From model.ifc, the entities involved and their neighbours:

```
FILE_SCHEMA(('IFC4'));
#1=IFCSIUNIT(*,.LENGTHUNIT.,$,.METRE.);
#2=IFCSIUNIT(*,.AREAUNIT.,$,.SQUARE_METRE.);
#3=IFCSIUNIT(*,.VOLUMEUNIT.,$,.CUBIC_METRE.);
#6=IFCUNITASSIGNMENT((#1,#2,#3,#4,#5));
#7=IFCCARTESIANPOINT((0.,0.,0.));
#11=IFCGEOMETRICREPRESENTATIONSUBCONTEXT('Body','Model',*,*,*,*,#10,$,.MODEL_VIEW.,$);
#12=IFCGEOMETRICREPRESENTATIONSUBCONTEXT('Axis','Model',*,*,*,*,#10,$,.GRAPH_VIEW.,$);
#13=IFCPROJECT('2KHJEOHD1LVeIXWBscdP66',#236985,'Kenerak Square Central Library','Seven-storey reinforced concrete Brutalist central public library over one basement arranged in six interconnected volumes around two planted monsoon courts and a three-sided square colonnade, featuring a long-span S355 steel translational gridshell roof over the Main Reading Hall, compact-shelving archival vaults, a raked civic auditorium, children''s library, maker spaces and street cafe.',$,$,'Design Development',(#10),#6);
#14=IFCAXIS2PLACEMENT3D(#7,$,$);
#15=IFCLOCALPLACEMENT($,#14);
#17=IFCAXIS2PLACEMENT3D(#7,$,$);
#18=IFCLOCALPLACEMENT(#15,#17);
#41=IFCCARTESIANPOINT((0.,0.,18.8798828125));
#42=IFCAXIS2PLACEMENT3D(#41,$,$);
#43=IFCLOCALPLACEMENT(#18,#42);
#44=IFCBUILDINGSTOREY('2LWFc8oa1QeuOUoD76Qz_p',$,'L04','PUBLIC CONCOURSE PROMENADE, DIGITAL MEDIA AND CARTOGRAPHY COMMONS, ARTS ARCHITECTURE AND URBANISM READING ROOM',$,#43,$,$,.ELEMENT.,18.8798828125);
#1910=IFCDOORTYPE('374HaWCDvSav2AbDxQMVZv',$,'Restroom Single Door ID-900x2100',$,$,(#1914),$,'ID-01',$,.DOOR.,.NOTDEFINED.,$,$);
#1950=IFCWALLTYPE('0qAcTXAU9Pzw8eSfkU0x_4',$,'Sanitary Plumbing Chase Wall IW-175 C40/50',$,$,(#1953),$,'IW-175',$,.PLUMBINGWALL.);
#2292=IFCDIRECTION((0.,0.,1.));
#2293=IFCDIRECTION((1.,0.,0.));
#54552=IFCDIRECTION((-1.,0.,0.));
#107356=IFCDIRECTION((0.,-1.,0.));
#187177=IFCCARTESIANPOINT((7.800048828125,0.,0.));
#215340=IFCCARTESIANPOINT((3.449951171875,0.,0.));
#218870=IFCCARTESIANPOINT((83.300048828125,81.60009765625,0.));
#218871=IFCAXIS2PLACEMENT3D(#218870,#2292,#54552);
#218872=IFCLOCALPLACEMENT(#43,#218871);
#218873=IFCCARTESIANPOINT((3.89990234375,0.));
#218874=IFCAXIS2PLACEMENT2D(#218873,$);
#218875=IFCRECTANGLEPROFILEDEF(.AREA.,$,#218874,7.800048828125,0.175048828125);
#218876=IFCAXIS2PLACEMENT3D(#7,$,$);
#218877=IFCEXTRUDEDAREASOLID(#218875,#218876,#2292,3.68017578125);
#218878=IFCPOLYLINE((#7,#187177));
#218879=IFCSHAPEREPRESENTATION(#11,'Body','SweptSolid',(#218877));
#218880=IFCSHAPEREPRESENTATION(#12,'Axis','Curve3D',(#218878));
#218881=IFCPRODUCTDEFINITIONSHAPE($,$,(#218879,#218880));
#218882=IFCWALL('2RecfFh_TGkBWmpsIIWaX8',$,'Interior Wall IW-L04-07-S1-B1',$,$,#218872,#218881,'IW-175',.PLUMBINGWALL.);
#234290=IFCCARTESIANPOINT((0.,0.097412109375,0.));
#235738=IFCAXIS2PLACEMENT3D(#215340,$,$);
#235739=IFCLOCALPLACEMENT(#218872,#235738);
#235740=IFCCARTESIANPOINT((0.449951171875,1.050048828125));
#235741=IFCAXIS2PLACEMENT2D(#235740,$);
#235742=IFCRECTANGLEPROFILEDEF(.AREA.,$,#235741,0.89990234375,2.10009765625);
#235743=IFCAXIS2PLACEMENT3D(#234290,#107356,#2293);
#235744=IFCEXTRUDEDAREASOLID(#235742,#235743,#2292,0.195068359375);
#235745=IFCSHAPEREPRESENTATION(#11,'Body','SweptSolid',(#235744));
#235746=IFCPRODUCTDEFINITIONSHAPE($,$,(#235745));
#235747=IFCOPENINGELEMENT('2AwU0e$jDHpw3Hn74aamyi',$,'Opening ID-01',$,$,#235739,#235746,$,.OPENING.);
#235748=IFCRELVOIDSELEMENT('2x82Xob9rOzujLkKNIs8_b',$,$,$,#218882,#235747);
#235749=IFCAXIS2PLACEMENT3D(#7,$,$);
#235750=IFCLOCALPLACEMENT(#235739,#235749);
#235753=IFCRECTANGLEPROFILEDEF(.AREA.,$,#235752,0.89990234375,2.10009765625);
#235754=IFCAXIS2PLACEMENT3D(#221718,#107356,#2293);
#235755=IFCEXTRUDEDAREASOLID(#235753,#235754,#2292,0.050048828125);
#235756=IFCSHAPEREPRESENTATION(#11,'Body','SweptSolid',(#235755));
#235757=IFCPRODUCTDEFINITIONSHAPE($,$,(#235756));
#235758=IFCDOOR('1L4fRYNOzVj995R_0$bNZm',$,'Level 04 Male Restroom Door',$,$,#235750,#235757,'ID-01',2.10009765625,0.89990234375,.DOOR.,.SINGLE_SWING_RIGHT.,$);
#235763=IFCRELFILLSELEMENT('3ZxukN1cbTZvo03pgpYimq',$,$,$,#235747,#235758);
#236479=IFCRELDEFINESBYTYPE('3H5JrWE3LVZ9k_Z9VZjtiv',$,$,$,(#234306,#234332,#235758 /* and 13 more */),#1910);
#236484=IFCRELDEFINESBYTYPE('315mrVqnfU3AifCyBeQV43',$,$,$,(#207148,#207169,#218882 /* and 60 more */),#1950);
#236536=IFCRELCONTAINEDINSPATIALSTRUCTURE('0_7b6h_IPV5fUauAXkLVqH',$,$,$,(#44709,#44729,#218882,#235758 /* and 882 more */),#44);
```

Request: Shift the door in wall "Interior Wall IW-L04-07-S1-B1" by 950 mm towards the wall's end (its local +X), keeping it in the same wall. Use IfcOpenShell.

```python
import ifcopenshell
import ifcopenshell.api.geometry
import ifcopenshell.util.placement

model = ifcopenshell.open("model.ifc")

door = model.by_guid("1L4fRYNOzVj995R_0$bNZm")
opening = door.FillsVoids[0].RelatingOpeningElement
wall = opening.VoidsElements[0].RelatingBuildingElement

wall_matrix = ifcopenshell.util.placement.get_local_placement(wall.ObjectPlacement)
shift = wall_matrix[:3, 0] * 0.95
before = ifcopenshell.util.placement.get_local_placement(door.ObjectPlacement)[:3, 3].copy()

# The door is placed relative to its opening, so it follows when the opening moves.
matrix = ifcopenshell.util.placement.get_local_placement(opening.ObjectPlacement)
matrix[:3, 3] += shift
ifcopenshell.api.geometry.edit_object_placement(
    model, product=opening, matrix=matrix, is_si=False, should_transform_children=True
)

after = ifcopenshell.util.placement.get_local_placement(door.ObjectPlacement)[:3, 3]
print("door moved by", (after - before).round(3) + 0.0)

model.write("model_updated.ifc")
```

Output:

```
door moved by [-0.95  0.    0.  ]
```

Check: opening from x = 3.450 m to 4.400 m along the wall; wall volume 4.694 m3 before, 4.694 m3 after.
